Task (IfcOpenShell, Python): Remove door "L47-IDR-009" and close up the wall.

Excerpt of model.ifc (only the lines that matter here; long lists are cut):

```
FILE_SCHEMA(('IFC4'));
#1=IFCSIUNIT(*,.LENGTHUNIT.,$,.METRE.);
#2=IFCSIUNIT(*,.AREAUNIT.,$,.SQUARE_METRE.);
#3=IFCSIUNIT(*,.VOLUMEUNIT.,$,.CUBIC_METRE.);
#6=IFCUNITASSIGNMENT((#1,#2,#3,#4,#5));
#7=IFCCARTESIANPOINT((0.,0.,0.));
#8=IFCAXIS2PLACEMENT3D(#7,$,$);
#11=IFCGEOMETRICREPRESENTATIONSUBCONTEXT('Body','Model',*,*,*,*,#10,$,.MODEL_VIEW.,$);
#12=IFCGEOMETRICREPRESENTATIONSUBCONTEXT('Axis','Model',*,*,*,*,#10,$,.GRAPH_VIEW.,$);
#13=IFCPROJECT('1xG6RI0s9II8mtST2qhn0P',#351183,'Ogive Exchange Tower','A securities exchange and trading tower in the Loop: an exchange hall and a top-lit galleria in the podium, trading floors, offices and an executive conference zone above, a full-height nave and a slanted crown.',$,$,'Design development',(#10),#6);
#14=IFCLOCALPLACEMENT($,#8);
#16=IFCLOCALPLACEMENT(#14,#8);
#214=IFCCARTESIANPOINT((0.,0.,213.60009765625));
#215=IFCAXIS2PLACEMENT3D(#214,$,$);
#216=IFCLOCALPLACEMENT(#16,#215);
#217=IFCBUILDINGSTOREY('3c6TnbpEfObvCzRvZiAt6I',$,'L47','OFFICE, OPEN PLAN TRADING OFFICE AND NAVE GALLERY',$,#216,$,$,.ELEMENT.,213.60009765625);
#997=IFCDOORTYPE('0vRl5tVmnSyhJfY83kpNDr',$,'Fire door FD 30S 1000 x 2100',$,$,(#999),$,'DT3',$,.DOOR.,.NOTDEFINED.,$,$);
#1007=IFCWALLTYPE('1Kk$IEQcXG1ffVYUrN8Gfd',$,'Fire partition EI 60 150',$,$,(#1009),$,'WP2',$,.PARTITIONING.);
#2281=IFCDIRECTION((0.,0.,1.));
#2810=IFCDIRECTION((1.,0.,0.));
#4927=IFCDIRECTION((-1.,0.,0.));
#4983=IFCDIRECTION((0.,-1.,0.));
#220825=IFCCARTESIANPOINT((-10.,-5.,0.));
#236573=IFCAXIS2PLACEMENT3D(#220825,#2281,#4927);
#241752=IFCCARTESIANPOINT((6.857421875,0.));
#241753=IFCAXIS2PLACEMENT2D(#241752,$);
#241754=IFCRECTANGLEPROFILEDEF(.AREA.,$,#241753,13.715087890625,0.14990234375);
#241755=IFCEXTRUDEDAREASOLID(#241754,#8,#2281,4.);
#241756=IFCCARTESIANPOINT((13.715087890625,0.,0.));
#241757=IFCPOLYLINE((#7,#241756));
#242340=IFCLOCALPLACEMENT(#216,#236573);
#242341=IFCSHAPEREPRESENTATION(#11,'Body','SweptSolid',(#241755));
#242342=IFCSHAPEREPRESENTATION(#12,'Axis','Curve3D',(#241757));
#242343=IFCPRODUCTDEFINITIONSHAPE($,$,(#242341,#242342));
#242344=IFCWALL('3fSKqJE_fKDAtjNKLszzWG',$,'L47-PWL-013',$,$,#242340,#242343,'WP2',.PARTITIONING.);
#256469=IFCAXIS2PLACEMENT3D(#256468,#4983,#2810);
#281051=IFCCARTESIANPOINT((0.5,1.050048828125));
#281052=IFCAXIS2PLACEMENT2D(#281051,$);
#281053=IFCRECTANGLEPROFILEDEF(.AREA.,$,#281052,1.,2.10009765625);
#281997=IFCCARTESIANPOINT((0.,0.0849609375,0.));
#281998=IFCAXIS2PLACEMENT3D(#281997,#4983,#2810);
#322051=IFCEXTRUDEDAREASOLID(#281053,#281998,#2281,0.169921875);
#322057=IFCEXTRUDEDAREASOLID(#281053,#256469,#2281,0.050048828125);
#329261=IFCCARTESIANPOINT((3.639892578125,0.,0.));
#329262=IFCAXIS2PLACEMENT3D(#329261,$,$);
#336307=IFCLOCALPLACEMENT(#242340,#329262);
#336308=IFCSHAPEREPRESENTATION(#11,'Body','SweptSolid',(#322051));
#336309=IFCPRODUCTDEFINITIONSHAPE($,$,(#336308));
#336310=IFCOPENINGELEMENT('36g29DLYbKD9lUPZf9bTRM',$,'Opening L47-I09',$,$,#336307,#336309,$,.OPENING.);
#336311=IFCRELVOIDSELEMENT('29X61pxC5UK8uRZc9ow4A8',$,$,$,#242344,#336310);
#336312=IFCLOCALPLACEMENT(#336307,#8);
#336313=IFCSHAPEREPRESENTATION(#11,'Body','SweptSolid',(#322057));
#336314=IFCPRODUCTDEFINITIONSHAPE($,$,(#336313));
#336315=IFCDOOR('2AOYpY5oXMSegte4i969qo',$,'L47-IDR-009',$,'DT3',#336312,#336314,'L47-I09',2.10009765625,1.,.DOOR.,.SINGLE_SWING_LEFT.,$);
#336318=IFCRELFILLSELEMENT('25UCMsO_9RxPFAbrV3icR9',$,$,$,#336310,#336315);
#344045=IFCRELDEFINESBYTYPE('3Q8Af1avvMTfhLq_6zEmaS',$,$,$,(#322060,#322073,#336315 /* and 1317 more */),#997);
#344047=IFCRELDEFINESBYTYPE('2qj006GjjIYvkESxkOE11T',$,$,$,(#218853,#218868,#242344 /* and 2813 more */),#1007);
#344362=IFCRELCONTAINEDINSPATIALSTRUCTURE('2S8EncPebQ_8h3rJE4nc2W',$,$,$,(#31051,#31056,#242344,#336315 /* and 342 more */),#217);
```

```python
import ifcopenshell
import ifcopenshell.api.feature
import ifcopenshell.api.root
import ifcopenshell.geom
import ifcopenshell.util.shape

model = ifcopenshell.open("model.ifc")
settings = ifcopenshell.geom.settings()


def volume(element):
    """Net volume in cubic metres, openings subtracted."""
    shape = ifcopenshell.geom.create_shape(settings, element)
    return ifcopenshell.util.shape.get_volume(shape.geometry)


door = model.by_guid("2AOYpY5oXMSegte4i969qo")
opening = door.FillsVoids[0].RelatingOpeningElement
wall = opening.VoidsElements[0].RelatingBuildingElement
before = volume(wall)

ifcopenshell.api.root.remove_product(model, product=door)
ifcopenshell.api.feature.remove_feature(model, feature=opening)

after = volume(wall)

print(f"wall volume {before:.3f} -> {after:.3f} m3")

model.write("model-out.ifc")
```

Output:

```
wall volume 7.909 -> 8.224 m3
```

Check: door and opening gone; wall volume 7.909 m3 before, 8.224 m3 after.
